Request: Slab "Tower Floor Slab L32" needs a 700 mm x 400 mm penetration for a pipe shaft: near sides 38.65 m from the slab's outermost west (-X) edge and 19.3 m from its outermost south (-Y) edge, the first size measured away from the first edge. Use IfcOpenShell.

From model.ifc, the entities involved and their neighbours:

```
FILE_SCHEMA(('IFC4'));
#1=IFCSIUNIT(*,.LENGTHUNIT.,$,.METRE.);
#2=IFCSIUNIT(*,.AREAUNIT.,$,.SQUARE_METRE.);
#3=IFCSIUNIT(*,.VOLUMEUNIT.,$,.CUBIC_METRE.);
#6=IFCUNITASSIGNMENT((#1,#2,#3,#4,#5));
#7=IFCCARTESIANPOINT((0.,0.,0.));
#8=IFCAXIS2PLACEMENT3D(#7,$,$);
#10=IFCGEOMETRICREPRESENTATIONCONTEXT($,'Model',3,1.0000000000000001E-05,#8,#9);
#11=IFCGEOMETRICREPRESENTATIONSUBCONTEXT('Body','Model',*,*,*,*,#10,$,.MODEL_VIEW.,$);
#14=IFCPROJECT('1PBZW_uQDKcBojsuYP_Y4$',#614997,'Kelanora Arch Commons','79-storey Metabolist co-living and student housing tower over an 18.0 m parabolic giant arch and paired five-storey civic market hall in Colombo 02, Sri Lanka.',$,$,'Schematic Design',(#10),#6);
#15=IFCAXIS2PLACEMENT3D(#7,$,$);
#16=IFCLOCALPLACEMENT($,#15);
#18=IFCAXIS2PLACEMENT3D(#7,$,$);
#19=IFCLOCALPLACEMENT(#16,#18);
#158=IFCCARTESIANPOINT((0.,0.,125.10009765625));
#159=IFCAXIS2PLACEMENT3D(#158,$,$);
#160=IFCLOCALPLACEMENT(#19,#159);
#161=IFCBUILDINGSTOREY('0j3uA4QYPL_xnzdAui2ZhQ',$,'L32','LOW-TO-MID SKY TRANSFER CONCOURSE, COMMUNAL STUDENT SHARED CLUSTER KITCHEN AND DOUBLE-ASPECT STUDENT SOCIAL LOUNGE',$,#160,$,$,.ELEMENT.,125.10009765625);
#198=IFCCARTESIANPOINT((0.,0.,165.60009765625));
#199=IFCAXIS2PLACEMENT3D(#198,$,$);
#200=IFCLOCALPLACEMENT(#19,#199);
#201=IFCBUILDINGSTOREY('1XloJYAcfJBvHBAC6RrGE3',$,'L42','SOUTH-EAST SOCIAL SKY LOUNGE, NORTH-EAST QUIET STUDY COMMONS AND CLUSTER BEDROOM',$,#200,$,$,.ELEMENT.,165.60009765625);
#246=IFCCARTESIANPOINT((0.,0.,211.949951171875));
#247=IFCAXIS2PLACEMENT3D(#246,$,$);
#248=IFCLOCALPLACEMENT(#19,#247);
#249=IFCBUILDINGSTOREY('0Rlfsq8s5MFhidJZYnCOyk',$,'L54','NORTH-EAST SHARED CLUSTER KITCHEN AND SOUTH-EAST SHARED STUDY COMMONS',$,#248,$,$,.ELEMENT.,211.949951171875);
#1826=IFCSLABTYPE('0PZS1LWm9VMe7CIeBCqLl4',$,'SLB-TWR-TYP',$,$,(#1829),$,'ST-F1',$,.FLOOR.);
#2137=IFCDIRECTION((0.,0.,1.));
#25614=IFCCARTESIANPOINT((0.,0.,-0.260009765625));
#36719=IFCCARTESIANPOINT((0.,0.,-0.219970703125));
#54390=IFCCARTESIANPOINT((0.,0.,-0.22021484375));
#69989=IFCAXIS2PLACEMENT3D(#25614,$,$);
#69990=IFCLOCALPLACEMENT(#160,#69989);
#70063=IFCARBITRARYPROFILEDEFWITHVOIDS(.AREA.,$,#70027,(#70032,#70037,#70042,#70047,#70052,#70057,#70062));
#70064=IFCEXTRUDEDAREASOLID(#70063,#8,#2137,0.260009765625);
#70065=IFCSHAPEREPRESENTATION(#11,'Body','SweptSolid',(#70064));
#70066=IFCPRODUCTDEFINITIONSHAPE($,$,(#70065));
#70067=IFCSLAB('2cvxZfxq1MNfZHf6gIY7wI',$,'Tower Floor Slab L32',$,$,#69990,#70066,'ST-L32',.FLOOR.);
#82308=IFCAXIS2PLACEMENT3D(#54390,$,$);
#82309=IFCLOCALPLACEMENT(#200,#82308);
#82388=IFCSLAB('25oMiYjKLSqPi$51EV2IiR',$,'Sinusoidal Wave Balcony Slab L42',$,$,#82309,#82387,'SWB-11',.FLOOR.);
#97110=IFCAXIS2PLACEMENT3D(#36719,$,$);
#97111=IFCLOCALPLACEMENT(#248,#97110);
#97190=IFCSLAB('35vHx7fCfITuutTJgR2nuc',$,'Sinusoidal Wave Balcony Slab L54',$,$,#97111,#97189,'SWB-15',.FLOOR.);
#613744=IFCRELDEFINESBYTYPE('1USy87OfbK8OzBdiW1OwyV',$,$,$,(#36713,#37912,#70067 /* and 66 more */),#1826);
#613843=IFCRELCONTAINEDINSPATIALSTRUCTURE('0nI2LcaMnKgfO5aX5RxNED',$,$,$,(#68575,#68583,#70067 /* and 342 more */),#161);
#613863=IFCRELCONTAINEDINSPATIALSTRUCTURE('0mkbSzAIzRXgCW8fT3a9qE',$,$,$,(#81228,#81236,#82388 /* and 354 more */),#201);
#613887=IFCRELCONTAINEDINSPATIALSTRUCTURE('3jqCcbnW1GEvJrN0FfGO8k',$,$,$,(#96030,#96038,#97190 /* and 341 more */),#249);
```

```python
import numpy as np
import ifcopenshell
import ifcopenshell.api.feature
import ifcopenshell.api.geometry
import ifcopenshell.api.root
import ifcopenshell.geom
import ifcopenshell.util.placement
import ifcopenshell.util.representation
import ifcopenshell.util.shape
import ifcopenshell.util.unit

model = ifcopenshell.open("model.ifc")
unit_scale = ifcopenshell.util.unit.calculate_unit_scale(model)
settings = ifcopenshell.geom.settings()


def volume(element):
    """Net volume in cubic metres, openings subtracted."""
    shape = ifcopenshell.geom.create_shape(settings, element)
    return ifcopenshell.util.shape.get_volume(shape.geometry)


slab = model.by_guid("2cvxZfxq1MNfZHf6gIY7wI")
before = volume(slab)

# Extent in the slab's own axes, in metres. The edges named are its -X and -Y sides.
slab_shape = ifcopenshell.geom.create_shape(settings, slab)
vertices = ifcopenshell.util.shape.get_vertices(slab_shape.geometry)
x_min, y_min, bottom = vertices.min(axis=0)
top = vertices[:, 2].max()

opening = ifcopenshell.api.root.create_entity(model, ifc_class="IfcOpeningElement", name="Pipe shaft opening", predefined_type="OPENING")
context = ifcopenshell.util.representation.get_context(model, "Model", "Body", "MODEL_VIEW")
width, depth = 0.7, 0.4
outline = [(0.0, 0.0), (width, 0.0), (width, depth), (0.0, depth), (0.0, 0.0)]
# Overshoot both faces by 50 mm so the cut is clean.
shape = ifcopenshell.api.geometry.add_slab_representation(
    model, context=context, depth=top - bottom + 0.1, polyline=outline
)
ifcopenshell.api.geometry.assign_representation(model, product=opening, representation=shape)

matrix = ifcopenshell.util.placement.get_local_placement(slab.ObjectPlacement)
matrix[:, 3] = matrix @ np.append(np.array([x_min + 38.65, y_min + 19.3, bottom - 0.05]) / unit_scale, 1.0)
ifcopenshell.api.geometry.edit_object_placement(model, product=opening, matrix=matrix, is_si=False)
ifcopenshell.api.feature.add_feature(model, feature=opening, element=slab)

after = volume(slab)

print(f"slab volume {before:.3f} -> {after:.3f} m3")

model.write("model_v2.ifc")
```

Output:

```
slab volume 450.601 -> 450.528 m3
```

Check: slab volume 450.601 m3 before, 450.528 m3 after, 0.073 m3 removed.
